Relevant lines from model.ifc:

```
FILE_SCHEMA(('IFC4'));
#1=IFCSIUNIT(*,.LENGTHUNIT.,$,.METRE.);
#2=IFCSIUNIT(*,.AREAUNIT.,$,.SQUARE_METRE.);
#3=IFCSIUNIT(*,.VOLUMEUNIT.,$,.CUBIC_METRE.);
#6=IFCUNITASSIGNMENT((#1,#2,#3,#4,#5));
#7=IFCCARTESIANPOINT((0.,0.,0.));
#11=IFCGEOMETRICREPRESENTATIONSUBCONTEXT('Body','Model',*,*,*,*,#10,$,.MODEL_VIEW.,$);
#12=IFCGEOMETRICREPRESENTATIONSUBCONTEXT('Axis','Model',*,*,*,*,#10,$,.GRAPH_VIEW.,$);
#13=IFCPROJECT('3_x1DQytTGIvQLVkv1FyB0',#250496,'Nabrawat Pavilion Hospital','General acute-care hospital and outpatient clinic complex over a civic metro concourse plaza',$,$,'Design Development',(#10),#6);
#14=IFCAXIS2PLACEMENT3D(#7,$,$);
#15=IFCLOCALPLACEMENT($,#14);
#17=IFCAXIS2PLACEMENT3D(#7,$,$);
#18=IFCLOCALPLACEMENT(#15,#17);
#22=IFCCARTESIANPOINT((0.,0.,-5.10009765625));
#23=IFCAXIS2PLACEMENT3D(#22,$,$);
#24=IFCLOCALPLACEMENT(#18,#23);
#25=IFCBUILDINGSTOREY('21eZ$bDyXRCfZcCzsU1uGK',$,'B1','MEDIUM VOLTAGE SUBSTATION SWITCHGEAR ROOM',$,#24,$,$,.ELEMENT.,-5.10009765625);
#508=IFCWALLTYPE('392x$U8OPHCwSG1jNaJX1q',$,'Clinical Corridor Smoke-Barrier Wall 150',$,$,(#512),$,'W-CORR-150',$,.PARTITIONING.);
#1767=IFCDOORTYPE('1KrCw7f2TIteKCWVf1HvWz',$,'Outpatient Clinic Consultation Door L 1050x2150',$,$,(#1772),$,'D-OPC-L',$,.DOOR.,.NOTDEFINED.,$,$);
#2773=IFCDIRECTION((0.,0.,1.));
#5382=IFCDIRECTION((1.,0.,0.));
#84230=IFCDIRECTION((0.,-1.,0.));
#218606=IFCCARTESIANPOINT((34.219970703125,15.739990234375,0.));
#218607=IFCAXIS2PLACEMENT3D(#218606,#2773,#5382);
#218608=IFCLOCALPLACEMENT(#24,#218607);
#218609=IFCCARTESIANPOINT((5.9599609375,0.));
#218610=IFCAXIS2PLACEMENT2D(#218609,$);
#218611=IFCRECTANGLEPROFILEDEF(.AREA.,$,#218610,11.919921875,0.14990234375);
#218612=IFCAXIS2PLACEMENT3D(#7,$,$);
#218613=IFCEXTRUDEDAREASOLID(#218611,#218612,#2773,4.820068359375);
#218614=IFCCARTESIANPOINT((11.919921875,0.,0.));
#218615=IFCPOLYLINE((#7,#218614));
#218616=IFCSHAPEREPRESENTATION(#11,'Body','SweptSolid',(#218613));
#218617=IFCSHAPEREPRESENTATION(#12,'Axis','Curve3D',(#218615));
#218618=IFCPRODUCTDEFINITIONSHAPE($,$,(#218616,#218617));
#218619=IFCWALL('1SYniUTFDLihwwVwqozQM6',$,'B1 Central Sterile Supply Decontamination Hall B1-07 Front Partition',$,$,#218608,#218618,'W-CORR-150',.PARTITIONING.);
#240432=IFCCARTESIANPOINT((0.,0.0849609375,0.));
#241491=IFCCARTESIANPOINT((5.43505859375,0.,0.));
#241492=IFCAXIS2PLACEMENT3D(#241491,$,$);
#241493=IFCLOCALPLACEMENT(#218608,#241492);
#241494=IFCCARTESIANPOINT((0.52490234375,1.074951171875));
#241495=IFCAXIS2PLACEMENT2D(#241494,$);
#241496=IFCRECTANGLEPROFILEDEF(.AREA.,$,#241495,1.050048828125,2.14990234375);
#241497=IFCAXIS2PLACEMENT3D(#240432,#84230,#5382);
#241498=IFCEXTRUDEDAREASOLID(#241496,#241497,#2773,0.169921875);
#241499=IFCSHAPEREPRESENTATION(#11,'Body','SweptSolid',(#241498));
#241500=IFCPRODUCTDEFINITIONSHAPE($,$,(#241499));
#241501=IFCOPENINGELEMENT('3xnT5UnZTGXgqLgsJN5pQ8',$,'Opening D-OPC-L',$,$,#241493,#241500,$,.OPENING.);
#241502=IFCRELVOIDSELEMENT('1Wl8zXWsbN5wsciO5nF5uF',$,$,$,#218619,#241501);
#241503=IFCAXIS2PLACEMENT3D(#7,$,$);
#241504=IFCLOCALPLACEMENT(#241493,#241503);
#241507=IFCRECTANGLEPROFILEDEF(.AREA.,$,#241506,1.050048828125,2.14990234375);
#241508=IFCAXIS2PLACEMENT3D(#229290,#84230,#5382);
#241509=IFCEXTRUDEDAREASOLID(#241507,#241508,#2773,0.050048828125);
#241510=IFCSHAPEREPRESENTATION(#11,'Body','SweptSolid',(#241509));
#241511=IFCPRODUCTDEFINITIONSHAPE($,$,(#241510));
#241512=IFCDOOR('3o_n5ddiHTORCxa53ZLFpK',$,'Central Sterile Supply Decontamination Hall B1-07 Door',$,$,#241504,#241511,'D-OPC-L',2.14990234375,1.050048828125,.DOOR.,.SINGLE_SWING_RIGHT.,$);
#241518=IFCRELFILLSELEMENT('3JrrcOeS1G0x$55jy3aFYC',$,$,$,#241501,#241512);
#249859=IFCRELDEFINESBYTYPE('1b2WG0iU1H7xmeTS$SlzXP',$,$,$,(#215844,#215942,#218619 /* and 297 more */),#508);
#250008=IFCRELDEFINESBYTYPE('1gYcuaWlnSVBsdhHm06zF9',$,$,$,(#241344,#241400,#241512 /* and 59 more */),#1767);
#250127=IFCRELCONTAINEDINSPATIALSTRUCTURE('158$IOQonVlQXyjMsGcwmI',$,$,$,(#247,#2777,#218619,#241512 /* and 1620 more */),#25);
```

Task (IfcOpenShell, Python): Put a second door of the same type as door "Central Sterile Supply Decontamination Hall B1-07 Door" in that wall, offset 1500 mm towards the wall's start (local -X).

```python
import ifcopenshell
import ifcopenshell.api.feature
import ifcopenshell.api.geometry
import ifcopenshell.api.root
import ifcopenshell.geom
import ifcopenshell.util.element
import ifcopenshell.util.placement
import ifcopenshell.util.shape

model = ifcopenshell.open("model.ifc")
settings = ifcopenshell.geom.settings()


def volume(element):
    """Net volume in cubic metres, openings subtracted."""
    shape = ifcopenshell.geom.create_shape(settings, element)
    return ifcopenshell.util.shape.get_volume(shape.geometry)


door = model.by_guid("3o_n5ddiHTORCxa53ZLFpK")
opening = door.FillsVoids[0].RelatingOpeningElement
wall = opening.VoidsElements[0].RelatingBuildingElement
before = volume(wall)
shift = ifcopenshell.util.placement.get_local_placement(wall.ObjectPlacement)[:3, 0] * -1.5

# copy_class copies the void relationship, type, container and properties, but no geometry.
new_opening = ifcopenshell.api.root.copy_class(model, product=opening)
new_opening.Representation = ifcopenshell.util.element.copy_deep(
    model, opening.Representation, exclude=["IfcGeometricRepresentationContext", "IfcRepresentationMap"]
)
new_door = ifcopenshell.api.root.copy_class(model, product=door)
new_door.Representation = ifcopenshell.util.element.copy_deep(
    model, door.Representation, exclude=["IfcGeometricRepresentationContext", "IfcRepresentationMap"]
)
new_door.Tag = None
ifcopenshell.api.feature.add_filling(model, opening=new_opening, element=new_door)

for old, new in ((opening, new_opening), (door, new_door)):
    matrix = ifcopenshell.util.placement.get_local_placement(old.ObjectPlacement)
    matrix[:3, 3] += shift
    ifcopenshell.api.geometry.edit_object_placement(model, product=new, matrix=matrix, is_si=False)

after = volume(wall)

print(f"wall volume {before:.3f} -> {after:.3f} m3")

model.write("model_updated.ifc")
```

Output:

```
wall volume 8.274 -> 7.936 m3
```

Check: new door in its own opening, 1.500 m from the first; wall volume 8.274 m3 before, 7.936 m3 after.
